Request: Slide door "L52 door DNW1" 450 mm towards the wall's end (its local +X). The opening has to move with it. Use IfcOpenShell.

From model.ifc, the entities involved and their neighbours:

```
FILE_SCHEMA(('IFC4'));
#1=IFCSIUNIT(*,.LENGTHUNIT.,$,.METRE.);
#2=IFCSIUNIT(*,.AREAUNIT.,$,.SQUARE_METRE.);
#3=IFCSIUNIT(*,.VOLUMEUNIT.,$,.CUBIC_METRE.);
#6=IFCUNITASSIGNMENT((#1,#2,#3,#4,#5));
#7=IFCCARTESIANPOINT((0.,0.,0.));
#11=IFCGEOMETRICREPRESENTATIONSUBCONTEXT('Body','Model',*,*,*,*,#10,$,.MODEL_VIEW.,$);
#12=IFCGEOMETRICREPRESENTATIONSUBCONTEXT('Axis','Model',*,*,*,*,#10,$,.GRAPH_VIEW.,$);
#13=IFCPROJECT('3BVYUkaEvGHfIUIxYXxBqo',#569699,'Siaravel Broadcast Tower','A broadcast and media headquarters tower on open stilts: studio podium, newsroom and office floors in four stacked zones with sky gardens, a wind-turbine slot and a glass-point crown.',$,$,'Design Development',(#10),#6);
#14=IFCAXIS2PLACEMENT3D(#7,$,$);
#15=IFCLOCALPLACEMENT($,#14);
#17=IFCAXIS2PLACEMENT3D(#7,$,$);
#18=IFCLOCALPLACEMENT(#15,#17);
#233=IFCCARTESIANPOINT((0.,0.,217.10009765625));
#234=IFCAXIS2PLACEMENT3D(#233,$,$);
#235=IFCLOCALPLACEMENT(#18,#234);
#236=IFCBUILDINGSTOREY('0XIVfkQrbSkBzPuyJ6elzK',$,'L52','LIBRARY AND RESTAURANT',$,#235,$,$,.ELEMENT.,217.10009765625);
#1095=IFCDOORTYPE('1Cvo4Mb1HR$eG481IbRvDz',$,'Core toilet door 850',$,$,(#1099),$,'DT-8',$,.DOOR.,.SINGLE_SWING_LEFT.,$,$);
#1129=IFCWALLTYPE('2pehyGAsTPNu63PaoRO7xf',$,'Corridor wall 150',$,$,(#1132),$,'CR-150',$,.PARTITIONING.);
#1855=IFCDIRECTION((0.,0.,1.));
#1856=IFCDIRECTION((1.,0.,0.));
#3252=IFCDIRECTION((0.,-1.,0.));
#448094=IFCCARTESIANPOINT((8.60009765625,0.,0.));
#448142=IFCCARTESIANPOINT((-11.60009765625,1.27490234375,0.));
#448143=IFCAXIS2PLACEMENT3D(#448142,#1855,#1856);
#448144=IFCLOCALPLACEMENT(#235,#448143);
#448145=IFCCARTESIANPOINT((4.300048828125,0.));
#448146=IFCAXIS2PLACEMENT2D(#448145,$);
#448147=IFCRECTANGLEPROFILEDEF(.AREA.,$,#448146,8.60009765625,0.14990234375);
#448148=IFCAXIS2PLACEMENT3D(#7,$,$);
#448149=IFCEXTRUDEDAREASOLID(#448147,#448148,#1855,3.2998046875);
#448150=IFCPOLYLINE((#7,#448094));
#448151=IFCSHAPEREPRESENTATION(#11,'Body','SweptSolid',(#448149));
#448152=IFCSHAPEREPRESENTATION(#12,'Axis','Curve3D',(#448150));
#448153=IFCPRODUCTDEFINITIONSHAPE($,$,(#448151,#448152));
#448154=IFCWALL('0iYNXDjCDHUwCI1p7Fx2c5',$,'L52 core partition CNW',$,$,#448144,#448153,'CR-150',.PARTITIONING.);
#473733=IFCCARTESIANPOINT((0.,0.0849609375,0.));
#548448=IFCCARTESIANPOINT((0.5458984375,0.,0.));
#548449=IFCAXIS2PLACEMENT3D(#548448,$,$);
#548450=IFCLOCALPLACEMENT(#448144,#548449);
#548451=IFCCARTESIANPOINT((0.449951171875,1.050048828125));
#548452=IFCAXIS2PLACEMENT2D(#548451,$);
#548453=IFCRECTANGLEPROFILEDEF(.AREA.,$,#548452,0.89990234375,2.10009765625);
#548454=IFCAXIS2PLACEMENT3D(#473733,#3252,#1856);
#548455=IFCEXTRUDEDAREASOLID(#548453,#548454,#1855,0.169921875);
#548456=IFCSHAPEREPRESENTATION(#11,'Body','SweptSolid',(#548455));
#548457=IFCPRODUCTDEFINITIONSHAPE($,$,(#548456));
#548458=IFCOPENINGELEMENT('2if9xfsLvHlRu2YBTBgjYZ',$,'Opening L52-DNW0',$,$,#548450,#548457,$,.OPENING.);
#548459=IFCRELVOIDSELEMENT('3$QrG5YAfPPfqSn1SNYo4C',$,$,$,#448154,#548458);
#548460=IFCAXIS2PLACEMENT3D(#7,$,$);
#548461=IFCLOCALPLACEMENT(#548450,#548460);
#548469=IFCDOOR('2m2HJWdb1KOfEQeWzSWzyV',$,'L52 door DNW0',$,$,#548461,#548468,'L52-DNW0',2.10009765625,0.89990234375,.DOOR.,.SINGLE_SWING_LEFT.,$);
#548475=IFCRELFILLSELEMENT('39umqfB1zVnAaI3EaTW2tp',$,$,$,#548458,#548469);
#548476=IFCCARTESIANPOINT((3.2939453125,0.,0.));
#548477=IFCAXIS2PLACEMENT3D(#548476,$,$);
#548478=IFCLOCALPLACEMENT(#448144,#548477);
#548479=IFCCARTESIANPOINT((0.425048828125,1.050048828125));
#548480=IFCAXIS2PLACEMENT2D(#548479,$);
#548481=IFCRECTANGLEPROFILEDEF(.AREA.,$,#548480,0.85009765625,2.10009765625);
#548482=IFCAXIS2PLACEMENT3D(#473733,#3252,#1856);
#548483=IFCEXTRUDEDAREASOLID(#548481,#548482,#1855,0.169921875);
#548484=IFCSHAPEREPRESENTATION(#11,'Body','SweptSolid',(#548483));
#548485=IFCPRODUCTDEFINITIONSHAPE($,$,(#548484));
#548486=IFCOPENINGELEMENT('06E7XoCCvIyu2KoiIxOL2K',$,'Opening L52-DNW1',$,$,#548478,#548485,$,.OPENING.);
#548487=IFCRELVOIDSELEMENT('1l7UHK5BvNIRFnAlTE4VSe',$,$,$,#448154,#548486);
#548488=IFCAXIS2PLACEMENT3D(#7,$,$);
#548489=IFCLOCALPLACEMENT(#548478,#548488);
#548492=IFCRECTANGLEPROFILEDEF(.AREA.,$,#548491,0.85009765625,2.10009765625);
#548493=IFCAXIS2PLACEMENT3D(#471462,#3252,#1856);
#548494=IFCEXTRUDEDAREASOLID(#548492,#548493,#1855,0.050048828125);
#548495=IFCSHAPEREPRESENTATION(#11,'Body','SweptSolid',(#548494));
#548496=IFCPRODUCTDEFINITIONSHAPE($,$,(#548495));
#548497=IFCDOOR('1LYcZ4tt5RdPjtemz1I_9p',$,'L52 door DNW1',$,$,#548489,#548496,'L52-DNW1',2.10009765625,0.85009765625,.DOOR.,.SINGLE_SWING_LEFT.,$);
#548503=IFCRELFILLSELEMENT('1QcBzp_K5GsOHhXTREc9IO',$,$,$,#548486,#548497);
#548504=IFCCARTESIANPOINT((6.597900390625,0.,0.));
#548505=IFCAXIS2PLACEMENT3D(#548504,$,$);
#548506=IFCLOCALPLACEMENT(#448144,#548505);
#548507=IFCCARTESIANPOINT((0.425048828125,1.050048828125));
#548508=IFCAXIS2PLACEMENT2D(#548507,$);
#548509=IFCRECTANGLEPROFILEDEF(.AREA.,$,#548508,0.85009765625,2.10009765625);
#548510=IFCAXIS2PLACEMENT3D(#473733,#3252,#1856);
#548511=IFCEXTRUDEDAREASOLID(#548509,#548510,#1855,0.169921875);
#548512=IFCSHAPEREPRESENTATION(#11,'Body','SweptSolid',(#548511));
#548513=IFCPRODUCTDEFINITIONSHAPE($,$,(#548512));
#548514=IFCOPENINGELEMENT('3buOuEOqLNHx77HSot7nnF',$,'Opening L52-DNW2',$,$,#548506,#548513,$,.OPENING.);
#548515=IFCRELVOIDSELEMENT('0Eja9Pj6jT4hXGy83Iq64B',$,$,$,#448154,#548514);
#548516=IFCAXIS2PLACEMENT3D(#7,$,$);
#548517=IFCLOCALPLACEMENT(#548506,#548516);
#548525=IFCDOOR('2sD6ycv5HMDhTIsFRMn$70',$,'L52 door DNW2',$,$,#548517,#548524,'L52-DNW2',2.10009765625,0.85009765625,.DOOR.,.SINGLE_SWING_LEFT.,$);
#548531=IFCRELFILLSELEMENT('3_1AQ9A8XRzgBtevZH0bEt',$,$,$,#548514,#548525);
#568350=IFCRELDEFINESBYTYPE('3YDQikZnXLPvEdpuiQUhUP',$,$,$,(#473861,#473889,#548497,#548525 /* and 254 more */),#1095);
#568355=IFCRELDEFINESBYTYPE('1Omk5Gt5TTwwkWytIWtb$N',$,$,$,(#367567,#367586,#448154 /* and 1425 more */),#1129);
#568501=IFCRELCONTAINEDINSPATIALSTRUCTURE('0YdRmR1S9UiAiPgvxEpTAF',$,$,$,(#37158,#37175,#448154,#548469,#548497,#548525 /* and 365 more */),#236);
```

```python
import ifcopenshell
import ifcopenshell.api.geometry
import ifcopenshell.util.placement
import ifcopenshell.util.unit

model = ifcopenshell.open("model.ifc")
unit_scale = ifcopenshell.util.unit.calculate_unit_scale(model)

door = model.by_guid("1LYcZ4tt5RdPjtemz1I_9p")
opening = door.FillsVoids[0].RelatingOpeningElement
wall = opening.VoidsElements[0].RelatingBuildingElement

wall_matrix = ifcopenshell.util.placement.get_local_placement(wall.ObjectPlacement)
shift = wall_matrix[:3, 0] * 0.45 / unit_scale
before = ifcopenshell.util.placement.get_local_placement(door.ObjectPlacement)[:3, 3].copy()

# The door is placed relative to its opening, so it follows when the opening moves.
matrix = ifcopenshell.util.placement.get_local_placement(opening.ObjectPlacement)
matrix[:3, 3] += shift
ifcopenshell.api.geometry.edit_object_placement(
    model, product=opening, matrix=matrix, is_si=False, should_transform_children=True
)

after = ifcopenshell.util.placement.get_local_placement(door.ObjectPlacement)[:3, 3]
print("door moved by", (after - before).round(3) + 0.0)

model.write("model_rev.ifc")
```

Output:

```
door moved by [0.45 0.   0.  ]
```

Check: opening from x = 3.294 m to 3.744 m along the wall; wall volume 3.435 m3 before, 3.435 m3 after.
